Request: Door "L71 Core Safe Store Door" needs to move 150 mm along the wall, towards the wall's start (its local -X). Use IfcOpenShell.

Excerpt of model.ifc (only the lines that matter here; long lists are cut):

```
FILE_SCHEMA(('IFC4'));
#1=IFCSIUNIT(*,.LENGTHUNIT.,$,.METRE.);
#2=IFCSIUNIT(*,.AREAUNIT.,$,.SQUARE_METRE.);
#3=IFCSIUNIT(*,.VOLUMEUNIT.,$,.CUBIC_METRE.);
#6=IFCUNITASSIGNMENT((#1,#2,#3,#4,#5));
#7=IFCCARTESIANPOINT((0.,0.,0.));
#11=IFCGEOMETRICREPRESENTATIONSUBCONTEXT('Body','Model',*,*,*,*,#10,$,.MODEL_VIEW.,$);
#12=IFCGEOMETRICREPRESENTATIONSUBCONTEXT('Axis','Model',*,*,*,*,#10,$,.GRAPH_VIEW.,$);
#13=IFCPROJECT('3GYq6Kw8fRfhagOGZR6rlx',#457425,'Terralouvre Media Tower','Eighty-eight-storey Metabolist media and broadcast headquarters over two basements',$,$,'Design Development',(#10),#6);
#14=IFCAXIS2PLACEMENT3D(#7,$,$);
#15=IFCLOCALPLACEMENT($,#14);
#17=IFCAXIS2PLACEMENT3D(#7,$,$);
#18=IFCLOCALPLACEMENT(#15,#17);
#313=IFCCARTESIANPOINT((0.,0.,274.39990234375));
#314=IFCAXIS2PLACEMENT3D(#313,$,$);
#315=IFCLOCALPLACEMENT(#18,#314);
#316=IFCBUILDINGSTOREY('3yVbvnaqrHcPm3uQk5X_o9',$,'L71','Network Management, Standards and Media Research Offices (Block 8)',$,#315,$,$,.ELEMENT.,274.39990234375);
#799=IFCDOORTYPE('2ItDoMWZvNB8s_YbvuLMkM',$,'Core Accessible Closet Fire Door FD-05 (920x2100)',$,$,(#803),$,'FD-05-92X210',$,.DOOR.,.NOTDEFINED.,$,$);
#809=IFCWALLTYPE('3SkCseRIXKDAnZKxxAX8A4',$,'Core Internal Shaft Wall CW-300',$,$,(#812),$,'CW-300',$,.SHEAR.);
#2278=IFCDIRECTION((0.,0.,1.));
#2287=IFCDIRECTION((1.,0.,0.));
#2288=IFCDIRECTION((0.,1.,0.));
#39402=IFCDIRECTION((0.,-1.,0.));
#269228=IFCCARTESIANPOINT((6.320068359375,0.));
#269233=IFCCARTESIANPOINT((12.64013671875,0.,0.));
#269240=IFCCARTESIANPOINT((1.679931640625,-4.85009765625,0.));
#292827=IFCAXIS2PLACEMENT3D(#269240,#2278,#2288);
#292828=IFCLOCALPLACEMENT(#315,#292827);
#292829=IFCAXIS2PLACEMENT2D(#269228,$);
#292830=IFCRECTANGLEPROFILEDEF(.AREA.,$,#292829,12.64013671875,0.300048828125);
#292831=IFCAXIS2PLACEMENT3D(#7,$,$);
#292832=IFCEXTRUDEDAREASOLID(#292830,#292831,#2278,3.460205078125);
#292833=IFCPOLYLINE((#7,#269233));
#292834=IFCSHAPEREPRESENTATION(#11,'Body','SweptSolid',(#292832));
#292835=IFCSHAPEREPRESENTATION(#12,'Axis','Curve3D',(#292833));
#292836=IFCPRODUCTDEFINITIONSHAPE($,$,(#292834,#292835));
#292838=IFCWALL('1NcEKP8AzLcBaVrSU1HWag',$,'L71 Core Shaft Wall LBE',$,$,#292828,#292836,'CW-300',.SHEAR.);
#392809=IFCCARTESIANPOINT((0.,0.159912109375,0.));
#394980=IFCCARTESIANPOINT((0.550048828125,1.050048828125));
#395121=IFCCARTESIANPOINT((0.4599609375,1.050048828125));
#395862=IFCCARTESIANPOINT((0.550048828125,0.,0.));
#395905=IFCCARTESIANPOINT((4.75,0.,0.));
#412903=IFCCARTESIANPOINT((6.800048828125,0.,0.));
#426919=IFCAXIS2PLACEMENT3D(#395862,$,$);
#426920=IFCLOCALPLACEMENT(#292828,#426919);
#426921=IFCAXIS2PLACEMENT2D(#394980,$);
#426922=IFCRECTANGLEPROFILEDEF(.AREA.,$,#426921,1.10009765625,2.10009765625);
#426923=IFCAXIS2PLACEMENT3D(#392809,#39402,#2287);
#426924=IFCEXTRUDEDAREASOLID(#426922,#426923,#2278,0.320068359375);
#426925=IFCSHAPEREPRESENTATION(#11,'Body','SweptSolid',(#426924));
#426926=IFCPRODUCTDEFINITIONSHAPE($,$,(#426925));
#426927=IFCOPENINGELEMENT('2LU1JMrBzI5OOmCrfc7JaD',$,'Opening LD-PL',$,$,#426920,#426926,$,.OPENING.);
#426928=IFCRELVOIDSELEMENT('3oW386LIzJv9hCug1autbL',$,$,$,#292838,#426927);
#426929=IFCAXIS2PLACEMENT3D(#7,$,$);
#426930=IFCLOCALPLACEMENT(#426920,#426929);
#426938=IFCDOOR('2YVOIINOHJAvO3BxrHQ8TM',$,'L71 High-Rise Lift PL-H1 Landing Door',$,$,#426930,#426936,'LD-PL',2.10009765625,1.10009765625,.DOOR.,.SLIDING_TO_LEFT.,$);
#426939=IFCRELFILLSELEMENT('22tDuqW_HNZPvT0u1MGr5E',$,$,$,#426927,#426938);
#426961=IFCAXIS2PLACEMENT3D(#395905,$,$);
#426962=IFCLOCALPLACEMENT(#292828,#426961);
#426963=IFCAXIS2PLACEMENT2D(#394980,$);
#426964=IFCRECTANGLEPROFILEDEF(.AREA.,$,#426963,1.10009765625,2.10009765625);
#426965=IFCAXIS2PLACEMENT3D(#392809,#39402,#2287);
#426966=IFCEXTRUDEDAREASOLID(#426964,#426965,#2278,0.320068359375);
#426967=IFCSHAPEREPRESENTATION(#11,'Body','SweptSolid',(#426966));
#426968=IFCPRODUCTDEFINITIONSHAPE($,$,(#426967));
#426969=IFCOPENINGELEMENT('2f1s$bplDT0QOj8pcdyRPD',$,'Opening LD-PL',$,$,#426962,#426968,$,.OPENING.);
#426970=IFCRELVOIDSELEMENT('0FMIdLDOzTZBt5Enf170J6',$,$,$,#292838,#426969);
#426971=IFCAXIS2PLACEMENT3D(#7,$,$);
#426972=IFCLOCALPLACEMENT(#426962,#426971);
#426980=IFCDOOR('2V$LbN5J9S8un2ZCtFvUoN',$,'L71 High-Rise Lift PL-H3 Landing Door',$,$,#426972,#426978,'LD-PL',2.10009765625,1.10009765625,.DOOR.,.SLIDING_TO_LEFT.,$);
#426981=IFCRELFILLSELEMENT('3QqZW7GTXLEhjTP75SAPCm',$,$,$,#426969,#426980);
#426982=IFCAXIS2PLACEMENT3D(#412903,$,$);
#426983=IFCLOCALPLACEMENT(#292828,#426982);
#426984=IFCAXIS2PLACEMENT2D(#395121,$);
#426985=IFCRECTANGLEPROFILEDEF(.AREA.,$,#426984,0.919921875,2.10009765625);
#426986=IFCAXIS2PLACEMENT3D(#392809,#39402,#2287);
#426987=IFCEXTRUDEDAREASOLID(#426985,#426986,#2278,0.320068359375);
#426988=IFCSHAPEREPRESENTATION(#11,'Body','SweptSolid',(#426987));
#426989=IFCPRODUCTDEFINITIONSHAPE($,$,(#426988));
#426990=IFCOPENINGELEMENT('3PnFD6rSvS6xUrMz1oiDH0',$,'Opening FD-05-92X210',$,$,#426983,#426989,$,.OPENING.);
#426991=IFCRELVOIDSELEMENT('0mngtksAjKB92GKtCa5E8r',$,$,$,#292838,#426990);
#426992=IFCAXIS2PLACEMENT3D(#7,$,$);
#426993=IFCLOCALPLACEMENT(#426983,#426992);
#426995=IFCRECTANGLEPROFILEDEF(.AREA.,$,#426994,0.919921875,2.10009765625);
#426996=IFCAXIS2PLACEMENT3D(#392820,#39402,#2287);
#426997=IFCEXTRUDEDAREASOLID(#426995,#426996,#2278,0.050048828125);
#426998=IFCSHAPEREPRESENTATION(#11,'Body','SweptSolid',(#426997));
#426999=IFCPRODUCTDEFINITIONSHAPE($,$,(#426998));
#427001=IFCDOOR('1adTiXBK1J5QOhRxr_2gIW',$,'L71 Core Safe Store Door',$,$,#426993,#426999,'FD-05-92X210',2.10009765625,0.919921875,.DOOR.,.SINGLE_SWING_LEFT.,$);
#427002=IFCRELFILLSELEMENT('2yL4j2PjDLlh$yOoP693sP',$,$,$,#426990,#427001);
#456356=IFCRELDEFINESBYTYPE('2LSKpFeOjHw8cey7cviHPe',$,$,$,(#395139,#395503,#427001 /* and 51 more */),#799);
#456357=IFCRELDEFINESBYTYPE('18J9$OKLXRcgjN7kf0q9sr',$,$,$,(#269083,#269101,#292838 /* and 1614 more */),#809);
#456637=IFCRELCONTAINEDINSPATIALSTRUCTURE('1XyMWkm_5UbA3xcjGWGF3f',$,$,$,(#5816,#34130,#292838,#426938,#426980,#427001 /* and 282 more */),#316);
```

```python
import ifcopenshell
import ifcopenshell.api.geometry
import ifcopenshell.util.placement
import ifcopenshell.util.unit

model = ifcopenshell.open("model.ifc")
unit_scale = ifcopenshell.util.unit.calculate_unit_scale(model)

door = model.by_guid("1adTiXBK1J5QOhRxr_2gIW")
opening = door.FillsVoids[0].RelatingOpeningElement
wall = opening.VoidsElements[0].RelatingBuildingElement

wall_matrix = ifcopenshell.util.placement.get_local_placement(wall.ObjectPlacement)
shift = wall_matrix[:3, 0] * -0.15 / unit_scale
before = ifcopenshell.util.placement.get_local_placement(door.ObjectPlacement)[:3, 3].copy()

# The door is placed relative to its opening, so it follows when the opening moves.
matrix = ifcopenshell.util.placement.get_local_placement(opening.ObjectPlacement)
matrix[:3, 3] += shift
ifcopenshell.api.geometry.edit_object_placement(
    model, product=opening, matrix=matrix, is_si=False, should_transform_children=True
)

after = ifcopenshell.util.placement.get_local_placement(door.ObjectPlacement)[:3, 3]
print("door moved by", (after - before).round(3) + 0.0)

model.write("model-out.ifc")
```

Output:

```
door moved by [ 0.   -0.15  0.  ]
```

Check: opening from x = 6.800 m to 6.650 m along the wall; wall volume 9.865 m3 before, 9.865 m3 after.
